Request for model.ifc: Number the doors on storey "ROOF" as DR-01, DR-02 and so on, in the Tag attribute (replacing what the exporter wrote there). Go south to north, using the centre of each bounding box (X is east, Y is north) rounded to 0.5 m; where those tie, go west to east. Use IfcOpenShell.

First a look at what the model holds.

```python
import ifcopenshell
import ifcopenshell.util.element
import ifcopenshell.util.placement

model = ifcopenshell.open("model.ifc")
print(model.schema)
storey = next(s for s in model.by_type("IfcBuildingStorey") if s.Name == "ROOF")
doors = [e for e in ifcopenshell.util.element.get_decomposition(storey) if e.is_a("IfcDoor")]
for e in sorted(doors, key=lambda e: e.id()):
    origin = ifcopenshell.util.placement.get_local_placement(e.ObjectPlacement)[:3, 3]
    print(e.id(), e.Tag, e.Name, origin.round(2) + 0.0, sep=" | ")
```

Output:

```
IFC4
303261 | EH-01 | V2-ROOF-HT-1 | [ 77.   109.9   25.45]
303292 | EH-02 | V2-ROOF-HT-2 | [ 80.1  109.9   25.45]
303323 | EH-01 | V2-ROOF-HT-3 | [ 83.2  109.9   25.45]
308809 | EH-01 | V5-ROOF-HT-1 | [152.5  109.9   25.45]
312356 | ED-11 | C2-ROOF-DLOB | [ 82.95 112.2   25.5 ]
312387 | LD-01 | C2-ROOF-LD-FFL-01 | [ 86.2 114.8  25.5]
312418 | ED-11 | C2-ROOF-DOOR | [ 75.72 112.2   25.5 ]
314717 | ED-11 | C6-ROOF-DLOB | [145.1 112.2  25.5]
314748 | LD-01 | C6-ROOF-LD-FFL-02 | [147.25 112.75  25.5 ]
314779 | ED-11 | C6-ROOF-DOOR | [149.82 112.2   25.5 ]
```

```python
import ifcopenshell
import ifcopenshell.geom
import ifcopenshell.util.element
import ifcopenshell.util.shape

model = ifcopenshell.open("model.ifc")
settings = ifcopenshell.geom.settings()
settings.set("use-world-coords", True)


def centre(element):
    shape = ifcopenshell.geom.create_shape(settings, element)
    return ifcopenshell.util.shape.get_bbox_centroid(shape.geometry)


storey = next(s for s in model.by_type("IfcBuildingStorey") if s.Name == "ROOF")
doors = [e for e in ifcopenshell.util.element.get_decomposition(storey) if e.is_a("IfcDoor")]

# Insertion points can sit at a corner or the storey origin, so sort by the geometry (in metres).
centres = {e: centre(e) for e in doors}
doors.sort(key=lambda e: (round(centres[e][1] / 0.5), centres[e][0]))

for i, e in enumerate(doors, start=1):
    number = f"DR-{i:02d}"
    e.Tag = number
    print(e.id(), number)

model.write("model_edited.ifc")
```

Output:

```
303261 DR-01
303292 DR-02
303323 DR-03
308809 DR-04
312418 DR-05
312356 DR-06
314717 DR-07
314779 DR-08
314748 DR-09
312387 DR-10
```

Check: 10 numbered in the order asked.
